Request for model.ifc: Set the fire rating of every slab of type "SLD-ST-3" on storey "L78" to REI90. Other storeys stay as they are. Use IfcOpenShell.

First a look at what the model holds.

```python
import ifcopenshell
import ifcopenshell.util.element

model = ifcopenshell.open("model.ifc")
print(model.schema)
storey = next(s for s in model.by_type("IfcBuildingStorey") if s.Name == "L78")
slabs = [e for e in ifcopenshell.util.element.get_decomposition(storey) if e.is_a("IfcSlab")]
seen = {}
for e in slabs:
    element_type = ifcopenshell.util.element.get_type(e)
    key = (element_type.Name if element_type != e and element_type else None, ifcopenshell.util.element.get_pset(e, "Pset_SlabCommon", "FireRating"))
    seen[key] = seen.get(key, 0) + 1
for (name, value), count in sorted(seen.items(), key=str):
    print(count, "x", name, "|", value)
```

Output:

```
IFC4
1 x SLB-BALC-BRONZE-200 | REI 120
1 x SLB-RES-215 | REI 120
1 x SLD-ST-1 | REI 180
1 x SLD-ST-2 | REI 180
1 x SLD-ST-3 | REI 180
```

```python
import ifcopenshell
import ifcopenshell.api.pset
import ifcopenshell.util.element

model = ifcopenshell.open("model.ifc")

storey = next(s for s in model.by_type("IfcBuildingStorey") if s.Name == "L78")
slabs = [e for e in ifcopenshell.util.element.get_decomposition(storey) if e.is_a("IfcSlab")]

count = 0
for e in slabs:
    element_type = ifcopenshell.util.element.get_type(e)
    if element_type in (None, e) or element_type.Name != "SLD-ST-3":
        continue
    found = ifcopenshell.util.element.get_pset(e, "Pset_SlabCommon", should_inherit=False)
    if found:
        pset = model.by_id(found["id"])
        if len(ifcopenshell.util.element.get_elements_by_pset(pset)) > 1:
            pset = ifcopenshell.api.pset.unshare_pset(model, products=[e], pset=pset)[0]
    else:
        pset = ifcopenshell.api.pset.add_pset(model, product=e, name="Pset_SlabCommon")
    ifcopenshell.api.pset.edit_pset(model, pset=pset, properties={"FireRating": "REI90"})
    count += 1

print(count, "slabs updated")

model.write("model-out.ifc")
```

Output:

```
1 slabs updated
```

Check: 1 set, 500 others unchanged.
